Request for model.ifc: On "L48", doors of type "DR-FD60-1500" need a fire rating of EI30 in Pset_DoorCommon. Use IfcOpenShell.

First a look at what the model holds.

```python
import ifcopenshell
import ifcopenshell.util.element

model = ifcopenshell.open("model.ifc")
print(model.schema)
storey = next(s for s in model.by_type("IfcBuildingStorey") if s.Name == "L48")
doors = [e for e in ifcopenshell.util.element.get_decomposition(storey) if e.is_a("IfcDoor")]
seen = {}
for e in doors:
    element_type = ifcopenshell.util.element.get_type(e)
    key = (element_type.Name if element_type != e and element_type else None, ifcopenshell.util.element.get_pset(e, "Pset_DoorCommon", "FireRating"))
    seen[key] = seen.get(key, 0) + 1
for (name, value), count in sorted(seen.items(), key=str):
    print(count, "x", name, "|", value)
```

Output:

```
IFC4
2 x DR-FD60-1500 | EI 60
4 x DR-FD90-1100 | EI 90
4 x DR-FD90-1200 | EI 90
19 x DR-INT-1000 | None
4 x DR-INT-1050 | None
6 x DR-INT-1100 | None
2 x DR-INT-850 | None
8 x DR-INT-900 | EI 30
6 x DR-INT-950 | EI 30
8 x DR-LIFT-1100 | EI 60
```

```python
import ifcopenshell
import ifcopenshell.api.pset
import ifcopenshell.util.element

model = ifcopenshell.open("model.ifc")

storey = next(s for s in model.by_type("IfcBuildingStorey") if s.Name == "L48")
doors = [e for e in ifcopenshell.util.element.get_decomposition(storey) if e.is_a("IfcDoor")]

count = 0
for e in doors:
    element_type = ifcopenshell.util.element.get_type(e)
    if element_type in (None, e) or element_type.Name != "DR-FD60-1500":
        continue
    # add_pset returns the element's existing set when there is one.
    pset = ifcopenshell.api.pset.add_pset(model, product=e, name="Pset_DoorCommon")
    ifcopenshell.api.pset.edit_pset(model, pset=pset, properties={"FireRating": "EI30"})
    count += 1

print(count, "doors updated")

model.write("model-out.ifc")
```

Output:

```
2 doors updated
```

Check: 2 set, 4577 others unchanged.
